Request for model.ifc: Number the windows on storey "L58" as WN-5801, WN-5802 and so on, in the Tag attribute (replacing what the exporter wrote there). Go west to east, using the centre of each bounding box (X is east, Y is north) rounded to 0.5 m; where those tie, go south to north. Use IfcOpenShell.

First a look at what the model holds.

```python
import ifcopenshell
import ifcopenshell.util.element
import ifcopenshell.util.placement

model = ifcopenshell.open("model.ifc")
print(model.schema)
storey = next(s for s in model.by_type("IfcBuildingStorey") if s.Name == "L58")
windows = [e for e in ifcopenshell.util.element.get_decomposition(storey) if e.is_a("IfcWindow")]
for e in sorted(windows, key=lambda e: e.id()):
    origin = ifcopenshell.util.placement.get_local_placement(e.ObjectPlacement)[:3, 3]
    print(e.id(), e.Tag, e.Name, origin.round(2) + 0.0, sep=" | ")
```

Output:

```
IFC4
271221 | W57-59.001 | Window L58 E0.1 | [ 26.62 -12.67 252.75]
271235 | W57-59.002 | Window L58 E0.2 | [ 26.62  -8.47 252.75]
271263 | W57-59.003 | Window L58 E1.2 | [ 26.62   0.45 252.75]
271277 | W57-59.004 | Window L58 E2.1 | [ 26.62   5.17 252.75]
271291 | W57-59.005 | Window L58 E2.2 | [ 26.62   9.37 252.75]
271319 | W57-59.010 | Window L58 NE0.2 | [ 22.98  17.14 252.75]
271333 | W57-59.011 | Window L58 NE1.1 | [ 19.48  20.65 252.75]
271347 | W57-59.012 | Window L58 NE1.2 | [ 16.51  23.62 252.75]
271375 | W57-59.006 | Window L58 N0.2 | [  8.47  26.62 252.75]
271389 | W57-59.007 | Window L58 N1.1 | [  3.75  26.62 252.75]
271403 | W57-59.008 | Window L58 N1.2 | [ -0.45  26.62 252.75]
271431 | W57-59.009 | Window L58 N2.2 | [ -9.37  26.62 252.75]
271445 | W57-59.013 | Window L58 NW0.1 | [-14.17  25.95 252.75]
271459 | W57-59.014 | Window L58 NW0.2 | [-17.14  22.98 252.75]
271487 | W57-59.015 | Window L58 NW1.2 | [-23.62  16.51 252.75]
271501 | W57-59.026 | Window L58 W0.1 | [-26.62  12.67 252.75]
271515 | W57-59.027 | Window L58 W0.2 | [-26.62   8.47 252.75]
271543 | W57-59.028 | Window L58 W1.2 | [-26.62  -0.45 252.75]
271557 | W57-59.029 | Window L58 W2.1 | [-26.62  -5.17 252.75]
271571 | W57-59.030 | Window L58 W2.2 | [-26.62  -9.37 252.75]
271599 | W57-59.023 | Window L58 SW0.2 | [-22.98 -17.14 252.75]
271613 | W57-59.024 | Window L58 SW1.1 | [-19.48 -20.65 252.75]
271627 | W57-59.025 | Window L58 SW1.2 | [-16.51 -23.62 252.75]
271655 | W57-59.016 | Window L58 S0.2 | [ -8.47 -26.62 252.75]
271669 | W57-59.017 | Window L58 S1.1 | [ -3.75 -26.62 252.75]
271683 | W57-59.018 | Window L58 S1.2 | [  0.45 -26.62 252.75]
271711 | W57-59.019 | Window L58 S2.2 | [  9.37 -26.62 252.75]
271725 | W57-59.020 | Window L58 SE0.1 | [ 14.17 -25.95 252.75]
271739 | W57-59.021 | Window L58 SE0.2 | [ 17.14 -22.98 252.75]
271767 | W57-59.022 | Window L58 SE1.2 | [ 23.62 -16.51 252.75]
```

```python
import ifcopenshell
import ifcopenshell.geom
import ifcopenshell.util.element
import ifcopenshell.util.shape

model = ifcopenshell.open("model.ifc")
settings = ifcopenshell.geom.settings()
settings.set("use-world-coords", True)


def centre(element):
    shape = ifcopenshell.geom.create_shape(settings, element)
    return ifcopenshell.util.shape.get_bbox_centroid(shape.geometry)


storey = next(s for s in model.by_type("IfcBuildingStorey") if s.Name == "L58")
windows = [e for e in ifcopenshell.util.element.get_decomposition(storey) if e.is_a("IfcWindow")]

# Insertion points can sit at a corner or the storey origin, so sort by the geometry (in metres).
centres = {e: centre(e) for e in windows}
windows.sort(key=lambda e: (round(centres[e][0] / 0.5), centres[e][1]))

for i, e in enumerate(windows, start=1):
    number = f"WN-58{i:02d}"
    e.Tag = number
    print(e.id(), number)

model.write("model_updated.ifc")
```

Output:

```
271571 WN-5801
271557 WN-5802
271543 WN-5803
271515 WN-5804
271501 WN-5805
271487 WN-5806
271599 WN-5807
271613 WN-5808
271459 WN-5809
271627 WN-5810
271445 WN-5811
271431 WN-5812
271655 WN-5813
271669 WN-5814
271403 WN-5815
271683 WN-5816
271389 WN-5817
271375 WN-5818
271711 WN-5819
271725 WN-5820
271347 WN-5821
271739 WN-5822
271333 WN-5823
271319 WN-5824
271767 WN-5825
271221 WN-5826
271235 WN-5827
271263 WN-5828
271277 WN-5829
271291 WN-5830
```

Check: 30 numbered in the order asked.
